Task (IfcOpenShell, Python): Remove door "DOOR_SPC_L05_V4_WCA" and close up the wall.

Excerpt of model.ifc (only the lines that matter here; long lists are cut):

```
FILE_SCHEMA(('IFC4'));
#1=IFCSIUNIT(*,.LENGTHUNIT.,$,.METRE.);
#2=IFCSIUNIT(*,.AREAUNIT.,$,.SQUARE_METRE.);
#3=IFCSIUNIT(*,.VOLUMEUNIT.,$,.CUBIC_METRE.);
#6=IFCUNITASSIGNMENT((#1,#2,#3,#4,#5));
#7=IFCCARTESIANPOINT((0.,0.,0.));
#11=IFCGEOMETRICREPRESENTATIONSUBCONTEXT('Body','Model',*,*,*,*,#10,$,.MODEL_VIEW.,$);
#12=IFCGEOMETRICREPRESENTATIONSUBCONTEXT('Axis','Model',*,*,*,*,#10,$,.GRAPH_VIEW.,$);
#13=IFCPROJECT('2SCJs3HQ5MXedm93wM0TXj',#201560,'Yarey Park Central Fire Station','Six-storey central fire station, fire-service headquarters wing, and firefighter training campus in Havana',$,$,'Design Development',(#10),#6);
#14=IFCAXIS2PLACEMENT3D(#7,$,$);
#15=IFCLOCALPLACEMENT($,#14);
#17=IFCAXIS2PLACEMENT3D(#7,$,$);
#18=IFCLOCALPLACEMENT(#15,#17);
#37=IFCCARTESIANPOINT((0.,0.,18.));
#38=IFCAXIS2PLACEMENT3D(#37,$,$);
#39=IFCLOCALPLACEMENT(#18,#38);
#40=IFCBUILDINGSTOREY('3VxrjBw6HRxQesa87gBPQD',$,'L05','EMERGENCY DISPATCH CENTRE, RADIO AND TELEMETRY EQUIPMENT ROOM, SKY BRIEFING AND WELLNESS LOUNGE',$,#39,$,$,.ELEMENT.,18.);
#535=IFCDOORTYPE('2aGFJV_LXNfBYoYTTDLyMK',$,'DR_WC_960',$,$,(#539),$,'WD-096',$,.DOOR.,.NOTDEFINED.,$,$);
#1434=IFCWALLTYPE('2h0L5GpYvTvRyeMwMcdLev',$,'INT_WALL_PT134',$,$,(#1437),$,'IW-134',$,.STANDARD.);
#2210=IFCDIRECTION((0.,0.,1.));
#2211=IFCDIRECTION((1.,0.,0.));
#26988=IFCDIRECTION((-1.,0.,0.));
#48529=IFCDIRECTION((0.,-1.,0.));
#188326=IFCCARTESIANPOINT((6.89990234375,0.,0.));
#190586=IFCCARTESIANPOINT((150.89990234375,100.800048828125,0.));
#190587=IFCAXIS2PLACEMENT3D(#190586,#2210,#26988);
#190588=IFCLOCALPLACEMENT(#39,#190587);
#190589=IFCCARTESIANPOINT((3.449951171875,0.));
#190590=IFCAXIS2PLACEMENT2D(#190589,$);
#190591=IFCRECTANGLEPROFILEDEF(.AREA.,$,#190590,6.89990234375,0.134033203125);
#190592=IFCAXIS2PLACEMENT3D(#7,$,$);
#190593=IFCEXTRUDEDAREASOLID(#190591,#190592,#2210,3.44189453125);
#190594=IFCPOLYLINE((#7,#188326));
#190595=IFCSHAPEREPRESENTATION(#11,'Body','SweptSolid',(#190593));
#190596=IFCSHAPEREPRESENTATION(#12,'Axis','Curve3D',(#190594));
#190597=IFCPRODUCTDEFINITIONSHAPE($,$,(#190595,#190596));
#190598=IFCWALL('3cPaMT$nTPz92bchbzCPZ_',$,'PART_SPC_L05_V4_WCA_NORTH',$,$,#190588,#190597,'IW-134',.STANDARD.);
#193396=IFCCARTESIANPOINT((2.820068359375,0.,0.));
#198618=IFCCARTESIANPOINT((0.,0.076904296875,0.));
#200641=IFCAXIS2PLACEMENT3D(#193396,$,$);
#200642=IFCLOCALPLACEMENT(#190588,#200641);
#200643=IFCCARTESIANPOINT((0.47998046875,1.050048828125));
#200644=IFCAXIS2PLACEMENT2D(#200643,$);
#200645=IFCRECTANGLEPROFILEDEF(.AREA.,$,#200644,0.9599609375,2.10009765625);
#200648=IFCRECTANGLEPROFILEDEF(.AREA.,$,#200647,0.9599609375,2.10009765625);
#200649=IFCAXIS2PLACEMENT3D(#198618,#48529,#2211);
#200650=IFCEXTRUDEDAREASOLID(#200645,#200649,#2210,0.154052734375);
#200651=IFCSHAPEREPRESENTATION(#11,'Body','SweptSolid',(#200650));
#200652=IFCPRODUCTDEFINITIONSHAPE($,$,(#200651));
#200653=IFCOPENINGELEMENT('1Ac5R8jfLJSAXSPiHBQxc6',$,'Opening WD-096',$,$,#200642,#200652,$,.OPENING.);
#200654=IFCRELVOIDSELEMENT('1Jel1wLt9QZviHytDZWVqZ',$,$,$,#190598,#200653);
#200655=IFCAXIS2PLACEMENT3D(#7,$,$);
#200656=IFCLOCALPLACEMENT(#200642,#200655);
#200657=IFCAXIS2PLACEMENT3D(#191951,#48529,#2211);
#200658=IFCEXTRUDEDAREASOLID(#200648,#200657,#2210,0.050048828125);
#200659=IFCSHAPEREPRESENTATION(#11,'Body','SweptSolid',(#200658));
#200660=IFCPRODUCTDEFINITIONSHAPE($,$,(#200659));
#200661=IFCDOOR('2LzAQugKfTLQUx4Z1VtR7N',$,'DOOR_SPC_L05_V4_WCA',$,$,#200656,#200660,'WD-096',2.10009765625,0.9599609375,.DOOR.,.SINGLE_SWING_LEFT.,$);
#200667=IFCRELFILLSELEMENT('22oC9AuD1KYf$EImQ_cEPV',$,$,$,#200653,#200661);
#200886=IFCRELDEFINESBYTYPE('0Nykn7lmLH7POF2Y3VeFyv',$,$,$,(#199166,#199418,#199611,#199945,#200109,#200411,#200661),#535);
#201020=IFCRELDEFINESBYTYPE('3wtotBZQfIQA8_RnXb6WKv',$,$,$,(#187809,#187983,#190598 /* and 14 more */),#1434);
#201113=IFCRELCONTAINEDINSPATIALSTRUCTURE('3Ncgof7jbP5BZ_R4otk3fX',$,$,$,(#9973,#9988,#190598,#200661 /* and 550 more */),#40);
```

```python
import ifcopenshell
import ifcopenshell.api.feature
import ifcopenshell.api.root
import ifcopenshell.geom
import ifcopenshell.util.shape

model = ifcopenshell.open("model.ifc")
settings = ifcopenshell.geom.settings()


def volume(element):
    """Net volume in cubic metres, openings subtracted."""
    shape = ifcopenshell.geom.create_shape(settings, element)
    return ifcopenshell.util.shape.get_volume(shape.geometry)


door = model.by_guid("2LzAQugKfTLQUx4Z1VtR7N")
opening = door.FillsVoids[0].RelatingOpeningElement
wall = opening.VoidsElements[0].RelatingBuildingElement
before = volume(wall)

ifcopenshell.api.root.remove_product(model, product=door)
ifcopenshell.api.feature.remove_feature(model, feature=opening)

after = volume(wall)

print(f"wall volume {before:.3f} -> {after:.3f} m3")

model.write("model-out.ifc")
```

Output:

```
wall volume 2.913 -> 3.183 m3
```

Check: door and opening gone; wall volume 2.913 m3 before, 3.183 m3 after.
